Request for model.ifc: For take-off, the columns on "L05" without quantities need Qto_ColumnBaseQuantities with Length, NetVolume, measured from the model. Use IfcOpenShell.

First a look at what the model holds.

```python
import ifcopenshell
import ifcopenshell.util.element
import ifcopenshell.util.unit

model = ifcopenshell.open("model.ifc")
print(model.schema)
for unit_type in ("LENGTHUNIT", "AREAUNIT", "VOLUMEUNIT"):
    print(unit_type, ifcopenshell.util.unit.calculate_unit_scale(model, unit_type))
storey = next(s for s in model.by_type("IfcBuildingStorey") if s.Name == "L05")
columns = [e for e in ifcopenshell.util.element.get_decomposition(storey) if e.is_a("IfcColumn")]
for e in sorted(columns, key=lambda e: e.id()):
    print(e.id(), e.is_a(), e.Name, list(ifcopenshell.util.element.get_psets(e, qtos_only=True)), sep=" | ")
```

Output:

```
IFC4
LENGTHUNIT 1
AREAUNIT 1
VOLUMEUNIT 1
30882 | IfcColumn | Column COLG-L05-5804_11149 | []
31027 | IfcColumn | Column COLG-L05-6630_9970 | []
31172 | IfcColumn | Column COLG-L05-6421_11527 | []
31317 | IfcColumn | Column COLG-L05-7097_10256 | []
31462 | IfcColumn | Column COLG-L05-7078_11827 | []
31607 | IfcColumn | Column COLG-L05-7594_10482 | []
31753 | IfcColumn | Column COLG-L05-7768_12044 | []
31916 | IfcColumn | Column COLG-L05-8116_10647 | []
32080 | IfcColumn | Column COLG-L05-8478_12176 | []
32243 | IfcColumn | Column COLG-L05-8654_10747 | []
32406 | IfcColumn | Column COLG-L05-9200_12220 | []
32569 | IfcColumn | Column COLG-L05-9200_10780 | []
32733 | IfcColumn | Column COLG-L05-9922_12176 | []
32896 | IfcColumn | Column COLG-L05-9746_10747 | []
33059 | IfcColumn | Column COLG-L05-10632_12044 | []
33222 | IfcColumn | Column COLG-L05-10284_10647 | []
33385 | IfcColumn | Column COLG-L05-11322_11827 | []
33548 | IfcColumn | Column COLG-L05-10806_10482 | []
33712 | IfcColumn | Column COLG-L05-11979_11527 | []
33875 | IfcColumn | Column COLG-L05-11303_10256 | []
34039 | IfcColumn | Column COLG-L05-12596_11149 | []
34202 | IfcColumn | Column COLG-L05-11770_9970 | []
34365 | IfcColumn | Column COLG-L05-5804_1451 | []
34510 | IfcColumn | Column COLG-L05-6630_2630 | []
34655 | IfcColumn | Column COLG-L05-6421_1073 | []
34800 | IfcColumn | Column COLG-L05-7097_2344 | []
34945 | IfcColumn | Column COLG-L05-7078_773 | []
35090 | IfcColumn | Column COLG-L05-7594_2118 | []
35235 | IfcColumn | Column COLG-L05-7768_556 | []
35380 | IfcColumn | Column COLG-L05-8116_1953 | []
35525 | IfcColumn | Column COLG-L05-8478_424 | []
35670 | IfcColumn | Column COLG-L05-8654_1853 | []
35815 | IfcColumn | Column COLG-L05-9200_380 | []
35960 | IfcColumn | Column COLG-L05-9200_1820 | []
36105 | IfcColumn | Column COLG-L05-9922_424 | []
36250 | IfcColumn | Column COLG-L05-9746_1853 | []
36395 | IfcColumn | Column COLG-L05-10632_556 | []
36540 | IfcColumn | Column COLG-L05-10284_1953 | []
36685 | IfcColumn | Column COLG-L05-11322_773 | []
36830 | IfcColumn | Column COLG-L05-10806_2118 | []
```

```python
import ifcopenshell
import ifcopenshell.api.pset
import ifcopenshell.geom
import ifcopenshell.util.element
import ifcopenshell.util.shape
import ifcopenshell.util.unit

model = ifcopenshell.open("model.ifc")
unit_scale = ifcopenshell.util.unit.calculate_unit_scale(model)
volume_scale = ifcopenshell.util.unit.calculate_unit_scale(model, "VOLUMEUNIT")
settings = ifcopenshell.geom.settings()

storey = next(s for s in model.by_type("IfcBuildingStorey") if s.Name == "L05")
columns = [e for e in ifcopenshell.util.element.get_decomposition(storey) if e.is_a("IfcColumn")]

for e in sorted(columns, key=lambda e: e.id()):
    if ifcopenshell.util.element.get_psets(e, qtos_only=True, should_inherit=False):
        continue
    # Geometry comes back in metres, in the element's own axes.
    shape = ifcopenshell.geom.create_shape(settings, e)
    values = {
        "Length": ifcopenshell.util.shape.get_z(shape.geometry) / unit_scale,
        "NetVolume": ifcopenshell.util.shape.get_volume(shape.geometry) / volume_scale,
    }
    qto = ifcopenshell.api.pset.add_qto(model, product=e, name="Qto_ColumnBaseQuantities")
    ifcopenshell.api.pset.edit_qto(model, qto=qto, properties=values)
    print(e.id(), {k: round(v, 3) for k, v in values.items()})

model.write("model_v2.ifc")
```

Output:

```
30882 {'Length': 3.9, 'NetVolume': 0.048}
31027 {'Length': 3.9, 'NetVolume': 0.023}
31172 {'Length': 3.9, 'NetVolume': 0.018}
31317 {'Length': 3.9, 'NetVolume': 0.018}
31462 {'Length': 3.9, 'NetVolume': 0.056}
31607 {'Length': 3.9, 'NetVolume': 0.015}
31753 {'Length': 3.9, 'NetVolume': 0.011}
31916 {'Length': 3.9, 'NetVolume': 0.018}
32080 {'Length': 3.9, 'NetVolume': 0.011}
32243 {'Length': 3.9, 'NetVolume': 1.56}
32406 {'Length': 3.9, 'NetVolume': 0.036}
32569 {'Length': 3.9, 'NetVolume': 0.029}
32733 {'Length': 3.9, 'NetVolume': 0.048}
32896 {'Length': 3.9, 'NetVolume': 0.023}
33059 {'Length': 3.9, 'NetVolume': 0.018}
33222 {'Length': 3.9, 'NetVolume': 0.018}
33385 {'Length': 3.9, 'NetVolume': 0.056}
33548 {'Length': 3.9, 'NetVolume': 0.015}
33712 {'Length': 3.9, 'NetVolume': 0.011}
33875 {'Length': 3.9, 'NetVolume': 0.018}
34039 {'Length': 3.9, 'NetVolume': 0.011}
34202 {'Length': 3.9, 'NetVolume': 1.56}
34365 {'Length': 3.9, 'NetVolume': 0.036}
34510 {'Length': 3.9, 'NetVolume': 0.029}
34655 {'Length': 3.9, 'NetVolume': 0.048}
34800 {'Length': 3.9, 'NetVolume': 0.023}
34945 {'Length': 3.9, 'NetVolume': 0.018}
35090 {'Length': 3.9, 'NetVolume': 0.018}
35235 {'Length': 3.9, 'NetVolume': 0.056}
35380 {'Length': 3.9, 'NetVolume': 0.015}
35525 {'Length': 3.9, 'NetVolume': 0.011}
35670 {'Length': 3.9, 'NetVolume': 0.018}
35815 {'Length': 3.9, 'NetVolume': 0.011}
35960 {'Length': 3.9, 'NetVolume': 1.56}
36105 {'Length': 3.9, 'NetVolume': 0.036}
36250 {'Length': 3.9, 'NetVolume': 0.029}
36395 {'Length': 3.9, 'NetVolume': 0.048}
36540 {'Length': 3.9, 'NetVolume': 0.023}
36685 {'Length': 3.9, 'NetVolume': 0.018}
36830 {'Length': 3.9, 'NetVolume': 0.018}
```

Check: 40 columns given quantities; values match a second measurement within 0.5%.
